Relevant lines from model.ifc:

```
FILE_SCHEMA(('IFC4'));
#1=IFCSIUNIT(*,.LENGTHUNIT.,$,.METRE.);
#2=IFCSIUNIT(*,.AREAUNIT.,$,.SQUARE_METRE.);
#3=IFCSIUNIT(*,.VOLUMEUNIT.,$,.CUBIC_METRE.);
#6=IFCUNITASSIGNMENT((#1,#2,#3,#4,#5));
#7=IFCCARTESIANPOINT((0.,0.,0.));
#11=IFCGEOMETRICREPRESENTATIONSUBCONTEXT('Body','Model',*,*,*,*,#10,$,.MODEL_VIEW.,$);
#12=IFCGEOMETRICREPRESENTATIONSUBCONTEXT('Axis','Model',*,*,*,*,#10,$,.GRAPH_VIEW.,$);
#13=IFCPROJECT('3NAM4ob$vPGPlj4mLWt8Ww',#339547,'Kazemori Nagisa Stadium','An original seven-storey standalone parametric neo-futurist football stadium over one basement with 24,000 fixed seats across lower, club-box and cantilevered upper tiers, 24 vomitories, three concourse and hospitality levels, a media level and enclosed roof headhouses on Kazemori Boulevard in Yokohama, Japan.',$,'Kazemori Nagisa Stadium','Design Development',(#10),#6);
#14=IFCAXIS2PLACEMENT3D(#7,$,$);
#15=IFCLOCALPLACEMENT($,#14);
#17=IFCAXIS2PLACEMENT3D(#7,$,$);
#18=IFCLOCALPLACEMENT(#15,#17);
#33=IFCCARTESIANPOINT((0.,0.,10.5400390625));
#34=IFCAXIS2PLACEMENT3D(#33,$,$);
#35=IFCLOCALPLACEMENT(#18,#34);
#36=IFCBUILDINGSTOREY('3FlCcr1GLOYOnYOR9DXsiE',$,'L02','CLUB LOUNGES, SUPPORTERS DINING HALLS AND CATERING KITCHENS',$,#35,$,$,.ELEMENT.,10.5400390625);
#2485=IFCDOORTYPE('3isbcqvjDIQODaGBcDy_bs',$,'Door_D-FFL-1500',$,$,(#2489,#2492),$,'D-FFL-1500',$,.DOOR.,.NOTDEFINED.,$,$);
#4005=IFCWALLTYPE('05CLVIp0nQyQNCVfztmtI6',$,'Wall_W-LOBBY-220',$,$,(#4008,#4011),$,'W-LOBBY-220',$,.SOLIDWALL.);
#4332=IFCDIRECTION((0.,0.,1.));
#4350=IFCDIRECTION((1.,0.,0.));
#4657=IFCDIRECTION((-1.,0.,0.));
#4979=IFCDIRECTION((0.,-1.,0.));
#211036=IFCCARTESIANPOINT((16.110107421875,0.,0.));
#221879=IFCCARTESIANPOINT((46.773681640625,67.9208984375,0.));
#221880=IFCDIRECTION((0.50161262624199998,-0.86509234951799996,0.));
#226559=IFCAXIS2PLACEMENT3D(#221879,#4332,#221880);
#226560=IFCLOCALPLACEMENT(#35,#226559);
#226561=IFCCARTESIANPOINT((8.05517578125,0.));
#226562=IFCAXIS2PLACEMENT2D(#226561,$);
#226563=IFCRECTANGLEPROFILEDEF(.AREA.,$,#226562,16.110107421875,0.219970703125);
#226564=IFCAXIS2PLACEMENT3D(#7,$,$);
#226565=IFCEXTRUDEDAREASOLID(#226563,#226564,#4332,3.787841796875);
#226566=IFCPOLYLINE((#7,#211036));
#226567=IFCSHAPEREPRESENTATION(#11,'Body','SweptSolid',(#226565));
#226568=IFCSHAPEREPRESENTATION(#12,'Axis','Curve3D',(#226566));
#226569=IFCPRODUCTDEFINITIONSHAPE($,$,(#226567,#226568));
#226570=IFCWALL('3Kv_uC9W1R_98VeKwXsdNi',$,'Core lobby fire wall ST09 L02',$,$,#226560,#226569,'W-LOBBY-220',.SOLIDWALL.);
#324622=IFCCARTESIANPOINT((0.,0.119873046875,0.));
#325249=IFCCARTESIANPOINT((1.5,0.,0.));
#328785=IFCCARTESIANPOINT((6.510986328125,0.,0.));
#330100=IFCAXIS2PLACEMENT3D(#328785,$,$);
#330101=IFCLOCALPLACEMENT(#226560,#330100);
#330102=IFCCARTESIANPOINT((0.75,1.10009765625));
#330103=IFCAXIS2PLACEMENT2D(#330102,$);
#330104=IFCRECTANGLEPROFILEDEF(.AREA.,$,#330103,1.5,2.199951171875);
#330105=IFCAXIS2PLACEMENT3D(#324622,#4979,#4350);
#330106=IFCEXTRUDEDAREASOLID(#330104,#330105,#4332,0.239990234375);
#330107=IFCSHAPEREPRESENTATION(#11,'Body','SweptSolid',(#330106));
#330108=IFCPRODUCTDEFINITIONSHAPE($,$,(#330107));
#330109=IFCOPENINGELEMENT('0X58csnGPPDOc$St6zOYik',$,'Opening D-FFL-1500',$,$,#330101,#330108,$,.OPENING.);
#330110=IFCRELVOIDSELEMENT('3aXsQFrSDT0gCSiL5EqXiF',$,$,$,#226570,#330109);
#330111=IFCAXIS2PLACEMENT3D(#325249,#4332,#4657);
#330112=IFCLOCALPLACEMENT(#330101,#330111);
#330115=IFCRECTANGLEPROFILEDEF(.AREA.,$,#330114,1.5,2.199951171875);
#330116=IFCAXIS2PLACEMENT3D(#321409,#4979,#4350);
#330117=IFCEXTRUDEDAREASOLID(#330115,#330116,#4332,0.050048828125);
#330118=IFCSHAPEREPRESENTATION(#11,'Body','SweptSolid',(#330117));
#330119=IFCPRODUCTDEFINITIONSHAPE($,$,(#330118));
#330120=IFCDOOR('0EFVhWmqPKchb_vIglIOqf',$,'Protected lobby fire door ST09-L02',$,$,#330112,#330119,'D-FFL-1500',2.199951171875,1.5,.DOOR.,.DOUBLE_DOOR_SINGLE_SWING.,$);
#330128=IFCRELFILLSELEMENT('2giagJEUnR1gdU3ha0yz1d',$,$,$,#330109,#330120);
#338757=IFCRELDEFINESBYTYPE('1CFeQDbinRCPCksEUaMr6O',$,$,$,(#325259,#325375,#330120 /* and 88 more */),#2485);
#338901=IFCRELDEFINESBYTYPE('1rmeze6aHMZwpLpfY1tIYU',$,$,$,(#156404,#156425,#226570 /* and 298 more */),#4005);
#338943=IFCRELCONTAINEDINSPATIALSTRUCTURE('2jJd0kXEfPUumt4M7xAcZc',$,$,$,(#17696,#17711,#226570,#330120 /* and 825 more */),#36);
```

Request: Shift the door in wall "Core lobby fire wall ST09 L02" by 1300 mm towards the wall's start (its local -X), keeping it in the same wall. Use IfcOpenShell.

```python
import ifcopenshell
import ifcopenshell.api.geometry
import ifcopenshell.util.placement

model = ifcopenshell.open("model.ifc")

door = model.by_guid("0EFVhWmqPKchb_vIglIOqf")
opening = door.FillsVoids[0].RelatingOpeningElement
wall = opening.VoidsElements[0].RelatingBuildingElement

wall_matrix = ifcopenshell.util.placement.get_local_placement(wall.ObjectPlacement)
shift = wall_matrix[:3, 0] * -1.3
before = ifcopenshell.util.placement.get_local_placement(door.ObjectPlacement)[:3, 3].copy()

# The door is placed relative to its opening, so it follows when the opening moves.
matrix = ifcopenshell.util.placement.get_local_placement(opening.ObjectPlacement)
matrix[:3, 3] += shift
ifcopenshell.api.geometry.edit_object_placement(
    model, product=opening, matrix=matrix, is_si=False, should_transform_children=True
)

after = ifcopenshell.util.placement.get_local_placement(door.ObjectPlacement)[:3, 3]
print("door moved by", (after - before).round(3) + 0.0)

model.write("model_updated.ifc")
```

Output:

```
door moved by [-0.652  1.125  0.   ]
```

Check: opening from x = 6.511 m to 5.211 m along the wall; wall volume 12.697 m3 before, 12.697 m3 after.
